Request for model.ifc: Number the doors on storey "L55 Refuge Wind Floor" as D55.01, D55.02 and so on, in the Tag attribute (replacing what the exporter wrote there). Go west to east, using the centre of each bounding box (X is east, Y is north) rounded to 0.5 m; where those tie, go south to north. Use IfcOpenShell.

First a look at what the model holds.

```python
import ifcopenshell
import ifcopenshell.util.element
import ifcopenshell.util.placement

model = ifcopenshell.open("model.ifc")
print(model.schema)
storey = next(s for s in model.by_type("IfcBuildingStorey") if s.Name == "L55 Refuge Wind Floor")
doors = [e for e in ifcopenshell.util.element.get_decomposition(storey) if e.is_a("IfcDoor")]
for e in sorted(doors, key=lambda e: e.id()):
    origin = ifcopenshell.util.placement.get_local_placement(e.ObjectPlacement)[:3, 3]
    print(e.id(), e.Tag, e.Name, origin.round(2) + 0.0, sep=" | ")
```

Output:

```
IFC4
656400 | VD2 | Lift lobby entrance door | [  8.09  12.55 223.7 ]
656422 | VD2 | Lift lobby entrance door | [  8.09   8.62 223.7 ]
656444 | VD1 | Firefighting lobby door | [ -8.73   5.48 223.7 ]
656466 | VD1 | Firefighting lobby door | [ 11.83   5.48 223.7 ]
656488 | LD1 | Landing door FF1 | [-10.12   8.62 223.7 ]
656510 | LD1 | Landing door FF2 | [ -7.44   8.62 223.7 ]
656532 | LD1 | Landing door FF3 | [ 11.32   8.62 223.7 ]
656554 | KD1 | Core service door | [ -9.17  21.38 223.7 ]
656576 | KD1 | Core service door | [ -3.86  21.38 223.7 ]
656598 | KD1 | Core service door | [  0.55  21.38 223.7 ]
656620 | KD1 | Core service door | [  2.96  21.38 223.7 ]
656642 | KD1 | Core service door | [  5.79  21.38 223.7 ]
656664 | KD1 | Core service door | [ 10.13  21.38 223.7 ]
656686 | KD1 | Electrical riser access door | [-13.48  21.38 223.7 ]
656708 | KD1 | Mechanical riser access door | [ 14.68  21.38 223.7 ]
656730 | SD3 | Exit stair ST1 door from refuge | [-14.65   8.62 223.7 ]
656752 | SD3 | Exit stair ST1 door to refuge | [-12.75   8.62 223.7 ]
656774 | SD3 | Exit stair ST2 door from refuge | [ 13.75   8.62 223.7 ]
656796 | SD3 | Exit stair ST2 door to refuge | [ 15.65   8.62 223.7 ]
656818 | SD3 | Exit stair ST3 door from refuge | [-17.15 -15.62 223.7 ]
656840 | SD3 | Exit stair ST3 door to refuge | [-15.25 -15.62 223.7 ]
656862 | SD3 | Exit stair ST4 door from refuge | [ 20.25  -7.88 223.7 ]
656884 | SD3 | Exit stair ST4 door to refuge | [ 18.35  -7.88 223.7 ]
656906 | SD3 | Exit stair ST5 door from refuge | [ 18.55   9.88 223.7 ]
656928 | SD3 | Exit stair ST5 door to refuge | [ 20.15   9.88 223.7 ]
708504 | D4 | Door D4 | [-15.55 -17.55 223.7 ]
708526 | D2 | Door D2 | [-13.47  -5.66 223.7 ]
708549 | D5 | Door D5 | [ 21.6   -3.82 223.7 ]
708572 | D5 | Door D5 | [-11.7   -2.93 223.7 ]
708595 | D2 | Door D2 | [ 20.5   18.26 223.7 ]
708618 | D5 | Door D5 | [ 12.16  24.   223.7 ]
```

```python
import ifcopenshell
import ifcopenshell.geom
import ifcopenshell.util.element
import ifcopenshell.util.shape

model = ifcopenshell.open("model.ifc")
settings = ifcopenshell.geom.settings()
settings.set("use-world-coords", True)


def centre(element):
    shape = ifcopenshell.geom.create_shape(settings, element)
    return ifcopenshell.util.shape.get_bbox_centroid(shape.geometry)


storey = next(s for s in model.by_type("IfcBuildingStorey") if s.Name == "L55 Refuge Wind Floor")
doors = [e for e in ifcopenshell.util.element.get_decomposition(storey) if e.is_a("IfcDoor")]

# Insertion points can sit at a corner or the storey origin, so sort by the geometry (in metres).
centres = {e: centre(e) for e in doors}
doors.sort(key=lambda e: (round(centres[e][0] / 0.5), centres[e][1]))

for i, e in enumerate(doors, start=1):
    number = f"D55.{i:02d}"
    e.Tag = number
    print(e.id(), number)

model.write("model_edited.ifc")
```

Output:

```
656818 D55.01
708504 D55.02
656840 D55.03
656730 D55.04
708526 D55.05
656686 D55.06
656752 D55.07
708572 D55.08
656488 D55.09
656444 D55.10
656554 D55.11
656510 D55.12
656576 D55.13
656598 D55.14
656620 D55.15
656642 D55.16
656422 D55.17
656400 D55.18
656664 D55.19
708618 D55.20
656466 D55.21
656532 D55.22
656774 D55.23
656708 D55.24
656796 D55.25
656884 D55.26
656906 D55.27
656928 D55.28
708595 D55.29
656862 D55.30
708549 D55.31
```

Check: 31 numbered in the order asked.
